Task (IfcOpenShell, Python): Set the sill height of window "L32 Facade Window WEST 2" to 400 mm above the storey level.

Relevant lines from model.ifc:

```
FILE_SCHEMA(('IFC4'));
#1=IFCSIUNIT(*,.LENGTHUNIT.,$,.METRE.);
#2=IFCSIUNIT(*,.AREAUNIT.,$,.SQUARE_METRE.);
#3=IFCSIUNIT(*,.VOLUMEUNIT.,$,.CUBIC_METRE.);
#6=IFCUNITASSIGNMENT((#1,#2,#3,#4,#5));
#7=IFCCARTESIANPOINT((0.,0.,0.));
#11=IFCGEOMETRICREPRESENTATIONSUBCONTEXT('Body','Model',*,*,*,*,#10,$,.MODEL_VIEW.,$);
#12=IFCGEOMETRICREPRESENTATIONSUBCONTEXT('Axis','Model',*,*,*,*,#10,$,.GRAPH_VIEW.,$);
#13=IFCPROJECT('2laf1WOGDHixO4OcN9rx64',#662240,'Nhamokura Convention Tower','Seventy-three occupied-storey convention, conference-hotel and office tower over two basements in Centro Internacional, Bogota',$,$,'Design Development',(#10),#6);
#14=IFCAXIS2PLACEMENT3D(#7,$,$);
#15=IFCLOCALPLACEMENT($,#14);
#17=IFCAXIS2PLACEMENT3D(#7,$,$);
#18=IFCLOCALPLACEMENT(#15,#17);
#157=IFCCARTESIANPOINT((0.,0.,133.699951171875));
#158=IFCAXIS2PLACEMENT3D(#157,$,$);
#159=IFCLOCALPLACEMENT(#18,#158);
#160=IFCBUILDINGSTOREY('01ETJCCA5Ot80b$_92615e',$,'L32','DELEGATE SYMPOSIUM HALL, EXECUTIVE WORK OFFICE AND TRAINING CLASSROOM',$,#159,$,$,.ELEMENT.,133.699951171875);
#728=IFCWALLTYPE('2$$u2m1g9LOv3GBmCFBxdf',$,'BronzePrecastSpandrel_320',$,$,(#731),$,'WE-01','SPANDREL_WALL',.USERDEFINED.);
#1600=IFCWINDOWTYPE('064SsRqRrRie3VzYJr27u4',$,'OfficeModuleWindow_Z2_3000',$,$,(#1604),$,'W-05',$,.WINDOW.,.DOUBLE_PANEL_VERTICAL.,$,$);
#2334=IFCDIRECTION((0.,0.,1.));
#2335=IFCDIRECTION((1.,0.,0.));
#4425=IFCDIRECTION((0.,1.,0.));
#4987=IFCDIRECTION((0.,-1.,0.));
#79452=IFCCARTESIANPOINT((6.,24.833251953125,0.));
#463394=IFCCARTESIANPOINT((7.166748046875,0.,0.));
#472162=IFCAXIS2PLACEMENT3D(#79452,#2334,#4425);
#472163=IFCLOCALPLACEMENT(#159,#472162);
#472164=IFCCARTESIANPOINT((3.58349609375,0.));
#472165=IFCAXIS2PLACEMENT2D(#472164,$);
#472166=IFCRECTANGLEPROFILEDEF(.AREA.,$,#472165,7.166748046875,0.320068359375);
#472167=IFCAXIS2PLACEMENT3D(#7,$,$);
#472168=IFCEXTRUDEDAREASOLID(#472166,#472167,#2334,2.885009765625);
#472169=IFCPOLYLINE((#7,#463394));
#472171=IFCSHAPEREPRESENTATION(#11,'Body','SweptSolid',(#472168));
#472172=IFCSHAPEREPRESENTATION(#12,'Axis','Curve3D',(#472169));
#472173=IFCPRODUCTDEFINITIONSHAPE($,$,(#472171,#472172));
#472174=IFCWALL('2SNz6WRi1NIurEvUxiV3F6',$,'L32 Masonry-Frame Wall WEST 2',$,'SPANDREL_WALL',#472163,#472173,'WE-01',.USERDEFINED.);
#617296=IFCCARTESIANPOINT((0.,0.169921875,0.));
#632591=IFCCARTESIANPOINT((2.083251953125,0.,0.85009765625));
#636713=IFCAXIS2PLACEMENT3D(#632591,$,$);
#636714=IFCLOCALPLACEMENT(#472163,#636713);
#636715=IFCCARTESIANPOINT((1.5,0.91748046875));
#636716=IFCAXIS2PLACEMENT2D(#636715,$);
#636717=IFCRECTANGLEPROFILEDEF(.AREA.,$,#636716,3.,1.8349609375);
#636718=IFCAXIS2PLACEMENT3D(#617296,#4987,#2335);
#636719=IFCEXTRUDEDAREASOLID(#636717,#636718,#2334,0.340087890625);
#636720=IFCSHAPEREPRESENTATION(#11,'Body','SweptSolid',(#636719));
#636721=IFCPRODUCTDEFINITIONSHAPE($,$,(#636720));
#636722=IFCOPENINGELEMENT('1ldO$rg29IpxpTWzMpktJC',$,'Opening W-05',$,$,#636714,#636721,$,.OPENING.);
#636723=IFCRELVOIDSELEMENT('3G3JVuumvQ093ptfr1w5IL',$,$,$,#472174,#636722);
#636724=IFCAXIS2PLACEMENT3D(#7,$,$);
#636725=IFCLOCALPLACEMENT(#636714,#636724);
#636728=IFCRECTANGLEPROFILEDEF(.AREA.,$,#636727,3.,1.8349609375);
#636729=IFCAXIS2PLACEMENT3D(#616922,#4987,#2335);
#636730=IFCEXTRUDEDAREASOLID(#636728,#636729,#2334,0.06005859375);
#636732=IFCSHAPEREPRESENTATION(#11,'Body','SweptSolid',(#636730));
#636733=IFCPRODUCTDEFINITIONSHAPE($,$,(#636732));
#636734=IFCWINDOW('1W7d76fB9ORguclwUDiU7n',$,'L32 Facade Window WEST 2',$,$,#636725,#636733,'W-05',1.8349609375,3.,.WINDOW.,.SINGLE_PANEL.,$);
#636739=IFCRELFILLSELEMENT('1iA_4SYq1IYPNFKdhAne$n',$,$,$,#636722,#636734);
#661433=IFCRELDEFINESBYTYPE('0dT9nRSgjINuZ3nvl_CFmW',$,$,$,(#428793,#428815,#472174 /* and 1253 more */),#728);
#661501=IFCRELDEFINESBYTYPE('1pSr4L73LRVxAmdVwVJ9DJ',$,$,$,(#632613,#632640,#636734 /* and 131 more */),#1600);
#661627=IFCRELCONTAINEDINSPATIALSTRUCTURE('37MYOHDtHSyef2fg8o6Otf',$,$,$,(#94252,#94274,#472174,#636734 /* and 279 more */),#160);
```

```python
import numpy as np
import ifcopenshell
import ifcopenshell.api.geometry
import ifcopenshell.geom
import ifcopenshell.util.element
import ifcopenshell.util.placement
import ifcopenshell.util.shape
import ifcopenshell.util.unit

model = ifcopenshell.open("model.ifc")
unit_scale = ifcopenshell.util.unit.calculate_unit_scale(model)

window = model.by_id(636734)
opening = window.FillsVoids[0].RelatingOpeningElement
storey = ifcopenshell.util.element.get_container(window, ifc_class="IfcBuildingStorey")
level = ifcopenshell.util.placement.get_local_placement(storey.ObjectPlacement)[2, 3]

# The opening's origin need not be at the sill, so measure its lowest point.
shape = ifcopenshell.geom.create_shape(ifcopenshell.geom.settings(), opening)
bottom = ifcopenshell.util.shape.get_shape_bottom_elevation(shape, shape.geometry) / unit_scale
dz = level + 0.4 / unit_scale - bottom

shift = np.array([0.0, 0.0, dz])
# The window is placed relative to its opening, so it follows when the opening moves.
matrix = ifcopenshell.util.placement.get_local_placement(opening.ObjectPlacement)
matrix[:3, 3] += shift
ifcopenshell.api.geometry.edit_object_placement(
    model, product=opening, matrix=matrix, is_si=False, should_transform_children=True
)

print(f"moved by {dz * unit_scale:+.3f} m")

model.write("model_edited.ifc")
```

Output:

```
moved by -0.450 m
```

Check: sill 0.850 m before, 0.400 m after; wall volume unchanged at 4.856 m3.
